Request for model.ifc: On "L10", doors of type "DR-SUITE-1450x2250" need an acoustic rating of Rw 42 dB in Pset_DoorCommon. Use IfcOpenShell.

First a look at what the model holds.

```python
import ifcopenshell
import ifcopenshell.util.element

model = ifcopenshell.open("model.ifc")
print(model.schema)
storey = next(s for s in model.by_type("IfcBuildingStorey") if s.Name == "L10")
doors = [e for e in ifcopenshell.util.element.get_decomposition(storey) if e.is_a("IfcDoor")]
seen = {}
for e in doors:
    element_type = ifcopenshell.util.element.get_type(e)
    key = (element_type.Name if element_type != e and element_type else None, ifcopenshell.util.element.get_pset(e, "Pset_DoorCommon", "AcousticRating"))
    seen[key] = seen.get(key, 0) + 1
for (name, value), count in sorted(seen.items(), key=str):
    print(count, "x", name, "|", value)
```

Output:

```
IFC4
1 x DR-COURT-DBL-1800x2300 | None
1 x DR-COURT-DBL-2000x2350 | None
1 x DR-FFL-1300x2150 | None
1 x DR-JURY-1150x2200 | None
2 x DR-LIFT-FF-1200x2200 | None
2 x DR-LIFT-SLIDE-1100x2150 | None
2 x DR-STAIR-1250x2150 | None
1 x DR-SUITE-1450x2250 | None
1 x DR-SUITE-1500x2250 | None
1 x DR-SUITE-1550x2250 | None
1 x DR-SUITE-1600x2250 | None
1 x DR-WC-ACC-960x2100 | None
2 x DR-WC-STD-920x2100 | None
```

```python
import ifcopenshell
import ifcopenshell.api.pset
import ifcopenshell.util.element

model = ifcopenshell.open("model.ifc")

storey = next(s for s in model.by_type("IfcBuildingStorey") if s.Name == "L10")
doors = [e for e in ifcopenshell.util.element.get_decomposition(storey) if e.is_a("IfcDoor")]

count = 0
for e in doors:
    element_type = ifcopenshell.util.element.get_type(e)
    if element_type in (None, e) or element_type.Name != "DR-SUITE-1450x2250":
        continue
    # add_pset returns the element's existing set when there is one.
    pset = ifcopenshell.api.pset.add_pset(model, product=e, name="Pset_DoorCommon")
    ifcopenshell.api.pset.edit_pset(model, pset=pset, properties={"AcousticRating": "Rw 42 dB"})
    count += 1

print(count, "doors updated")

model.write("model_v2.ifc")
```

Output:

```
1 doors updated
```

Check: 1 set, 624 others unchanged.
